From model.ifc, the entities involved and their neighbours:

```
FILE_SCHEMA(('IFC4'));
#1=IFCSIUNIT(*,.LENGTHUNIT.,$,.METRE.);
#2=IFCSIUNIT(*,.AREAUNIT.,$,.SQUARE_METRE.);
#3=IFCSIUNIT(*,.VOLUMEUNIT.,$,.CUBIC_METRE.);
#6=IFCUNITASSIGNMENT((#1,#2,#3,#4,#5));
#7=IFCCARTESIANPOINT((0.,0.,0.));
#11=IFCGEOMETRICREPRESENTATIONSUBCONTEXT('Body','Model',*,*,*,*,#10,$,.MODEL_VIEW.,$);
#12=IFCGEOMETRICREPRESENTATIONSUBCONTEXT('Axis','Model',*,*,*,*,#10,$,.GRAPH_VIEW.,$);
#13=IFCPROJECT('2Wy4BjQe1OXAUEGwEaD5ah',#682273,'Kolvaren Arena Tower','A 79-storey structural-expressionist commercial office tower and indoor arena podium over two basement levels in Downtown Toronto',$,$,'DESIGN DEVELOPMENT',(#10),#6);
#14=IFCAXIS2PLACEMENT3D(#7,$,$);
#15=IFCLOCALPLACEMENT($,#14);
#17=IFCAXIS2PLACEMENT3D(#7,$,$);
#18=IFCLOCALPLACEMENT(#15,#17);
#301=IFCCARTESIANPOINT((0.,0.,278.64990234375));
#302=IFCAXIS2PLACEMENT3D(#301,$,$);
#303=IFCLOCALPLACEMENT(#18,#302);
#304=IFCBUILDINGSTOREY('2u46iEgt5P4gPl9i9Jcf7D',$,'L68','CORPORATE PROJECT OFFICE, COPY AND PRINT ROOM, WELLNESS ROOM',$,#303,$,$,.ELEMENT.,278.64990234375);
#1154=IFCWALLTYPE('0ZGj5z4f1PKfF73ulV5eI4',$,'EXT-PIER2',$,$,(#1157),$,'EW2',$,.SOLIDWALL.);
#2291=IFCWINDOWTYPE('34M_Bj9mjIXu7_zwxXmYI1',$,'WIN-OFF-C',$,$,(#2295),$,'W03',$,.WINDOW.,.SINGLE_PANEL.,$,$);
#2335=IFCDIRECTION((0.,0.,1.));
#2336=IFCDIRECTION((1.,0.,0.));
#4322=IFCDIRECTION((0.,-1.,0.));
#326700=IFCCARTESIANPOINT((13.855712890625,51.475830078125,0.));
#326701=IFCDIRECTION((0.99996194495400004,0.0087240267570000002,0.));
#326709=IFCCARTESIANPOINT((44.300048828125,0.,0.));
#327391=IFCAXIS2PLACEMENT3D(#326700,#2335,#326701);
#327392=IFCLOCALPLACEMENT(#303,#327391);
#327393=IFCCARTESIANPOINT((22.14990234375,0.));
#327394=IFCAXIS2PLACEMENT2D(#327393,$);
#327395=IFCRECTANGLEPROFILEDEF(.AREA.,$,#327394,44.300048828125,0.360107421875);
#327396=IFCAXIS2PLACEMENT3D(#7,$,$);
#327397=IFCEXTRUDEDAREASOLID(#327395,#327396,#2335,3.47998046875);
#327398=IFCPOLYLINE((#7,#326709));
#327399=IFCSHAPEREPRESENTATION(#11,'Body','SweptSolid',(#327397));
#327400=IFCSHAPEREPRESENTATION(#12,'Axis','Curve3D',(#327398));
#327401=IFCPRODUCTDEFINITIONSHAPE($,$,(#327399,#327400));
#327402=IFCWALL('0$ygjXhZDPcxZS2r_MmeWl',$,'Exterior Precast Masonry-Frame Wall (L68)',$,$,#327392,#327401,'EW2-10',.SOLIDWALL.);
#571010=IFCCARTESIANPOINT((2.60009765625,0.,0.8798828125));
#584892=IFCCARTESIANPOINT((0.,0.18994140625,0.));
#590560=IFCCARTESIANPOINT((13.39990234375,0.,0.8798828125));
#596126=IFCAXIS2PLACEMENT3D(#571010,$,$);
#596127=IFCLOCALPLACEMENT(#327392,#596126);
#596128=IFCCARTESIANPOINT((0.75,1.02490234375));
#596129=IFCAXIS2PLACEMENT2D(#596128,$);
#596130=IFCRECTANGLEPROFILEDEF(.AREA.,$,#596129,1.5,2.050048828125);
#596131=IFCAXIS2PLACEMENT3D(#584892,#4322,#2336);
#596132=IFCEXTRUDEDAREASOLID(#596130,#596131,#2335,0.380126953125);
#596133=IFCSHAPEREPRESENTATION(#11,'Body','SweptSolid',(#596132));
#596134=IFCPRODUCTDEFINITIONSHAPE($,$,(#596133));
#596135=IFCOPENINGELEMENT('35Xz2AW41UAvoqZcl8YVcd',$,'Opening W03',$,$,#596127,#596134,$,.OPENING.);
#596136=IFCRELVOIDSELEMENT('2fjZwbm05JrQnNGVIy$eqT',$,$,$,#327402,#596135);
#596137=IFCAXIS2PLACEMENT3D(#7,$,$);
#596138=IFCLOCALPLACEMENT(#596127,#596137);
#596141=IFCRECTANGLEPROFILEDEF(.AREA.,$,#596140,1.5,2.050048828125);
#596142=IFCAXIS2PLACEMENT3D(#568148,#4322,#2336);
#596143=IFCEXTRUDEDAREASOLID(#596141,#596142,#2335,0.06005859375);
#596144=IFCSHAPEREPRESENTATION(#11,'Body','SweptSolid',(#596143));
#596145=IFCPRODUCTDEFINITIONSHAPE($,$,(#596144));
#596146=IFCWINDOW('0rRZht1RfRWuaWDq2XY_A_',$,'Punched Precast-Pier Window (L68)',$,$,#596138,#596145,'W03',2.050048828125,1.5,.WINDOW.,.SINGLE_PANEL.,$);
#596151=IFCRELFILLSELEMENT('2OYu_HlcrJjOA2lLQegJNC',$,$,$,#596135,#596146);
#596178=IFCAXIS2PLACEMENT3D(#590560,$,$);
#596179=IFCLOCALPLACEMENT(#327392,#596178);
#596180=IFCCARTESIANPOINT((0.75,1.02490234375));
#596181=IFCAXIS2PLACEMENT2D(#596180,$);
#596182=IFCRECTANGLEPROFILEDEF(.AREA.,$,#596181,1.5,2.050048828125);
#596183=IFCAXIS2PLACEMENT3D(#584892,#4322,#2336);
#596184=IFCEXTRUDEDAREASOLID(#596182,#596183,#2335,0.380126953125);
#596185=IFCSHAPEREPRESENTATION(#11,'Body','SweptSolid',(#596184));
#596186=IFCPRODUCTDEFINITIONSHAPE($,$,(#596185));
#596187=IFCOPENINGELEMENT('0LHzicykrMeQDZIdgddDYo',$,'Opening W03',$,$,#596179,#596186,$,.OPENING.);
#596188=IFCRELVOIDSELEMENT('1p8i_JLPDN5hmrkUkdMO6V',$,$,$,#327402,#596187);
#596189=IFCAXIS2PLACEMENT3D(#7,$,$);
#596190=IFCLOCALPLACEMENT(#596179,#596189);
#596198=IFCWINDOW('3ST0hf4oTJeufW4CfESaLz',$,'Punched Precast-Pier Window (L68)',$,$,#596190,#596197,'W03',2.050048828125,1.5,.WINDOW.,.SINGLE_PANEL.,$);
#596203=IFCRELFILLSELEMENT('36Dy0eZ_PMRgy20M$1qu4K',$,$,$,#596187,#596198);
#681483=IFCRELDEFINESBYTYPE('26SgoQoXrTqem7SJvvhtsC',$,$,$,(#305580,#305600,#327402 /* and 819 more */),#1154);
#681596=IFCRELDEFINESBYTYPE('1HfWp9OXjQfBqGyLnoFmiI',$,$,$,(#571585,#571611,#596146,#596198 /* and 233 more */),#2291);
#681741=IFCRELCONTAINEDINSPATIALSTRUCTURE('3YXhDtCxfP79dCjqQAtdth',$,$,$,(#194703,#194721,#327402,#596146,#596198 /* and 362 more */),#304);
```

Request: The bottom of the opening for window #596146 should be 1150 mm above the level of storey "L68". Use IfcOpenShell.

```python
import numpy as np
import ifcopenshell
import ifcopenshell.api.geometry
import ifcopenshell.geom
import ifcopenshell.util.element
import ifcopenshell.util.placement
import ifcopenshell.util.shape
import ifcopenshell.util.unit

model = ifcopenshell.open("model.ifc")
unit_scale = ifcopenshell.util.unit.calculate_unit_scale(model)

window = model.by_guid("0rRZht1RfRWuaWDq2XY_A_")
opening = window.FillsVoids[0].RelatingOpeningElement
storey = ifcopenshell.util.element.get_container(window, ifc_class="IfcBuildingStorey")
level = ifcopenshell.util.placement.get_local_placement(storey.ObjectPlacement)[2, 3]

# The opening's origin need not be at the sill, so measure its lowest point.
shape = ifcopenshell.geom.create_shape(ifcopenshell.geom.settings(), opening)
bottom = ifcopenshell.util.shape.get_shape_bottom_elevation(shape, shape.geometry) / unit_scale
dz = level + 1.15 / unit_scale - bottom

shift = np.array([0.0, 0.0, dz])
# The window is placed relative to its opening, so it follows when the opening moves.
matrix = ifcopenshell.util.placement.get_local_placement(opening.ObjectPlacement)
matrix[:3, 3] += shift
ifcopenshell.api.geometry.edit_object_placement(
    model, product=opening, matrix=matrix, is_si=False, should_transform_children=True
)

print(f"moved by {dz * unit_scale:+.3f} m")

model.write("model_edited.ifc")
```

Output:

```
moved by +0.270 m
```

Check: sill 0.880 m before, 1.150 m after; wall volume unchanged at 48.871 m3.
